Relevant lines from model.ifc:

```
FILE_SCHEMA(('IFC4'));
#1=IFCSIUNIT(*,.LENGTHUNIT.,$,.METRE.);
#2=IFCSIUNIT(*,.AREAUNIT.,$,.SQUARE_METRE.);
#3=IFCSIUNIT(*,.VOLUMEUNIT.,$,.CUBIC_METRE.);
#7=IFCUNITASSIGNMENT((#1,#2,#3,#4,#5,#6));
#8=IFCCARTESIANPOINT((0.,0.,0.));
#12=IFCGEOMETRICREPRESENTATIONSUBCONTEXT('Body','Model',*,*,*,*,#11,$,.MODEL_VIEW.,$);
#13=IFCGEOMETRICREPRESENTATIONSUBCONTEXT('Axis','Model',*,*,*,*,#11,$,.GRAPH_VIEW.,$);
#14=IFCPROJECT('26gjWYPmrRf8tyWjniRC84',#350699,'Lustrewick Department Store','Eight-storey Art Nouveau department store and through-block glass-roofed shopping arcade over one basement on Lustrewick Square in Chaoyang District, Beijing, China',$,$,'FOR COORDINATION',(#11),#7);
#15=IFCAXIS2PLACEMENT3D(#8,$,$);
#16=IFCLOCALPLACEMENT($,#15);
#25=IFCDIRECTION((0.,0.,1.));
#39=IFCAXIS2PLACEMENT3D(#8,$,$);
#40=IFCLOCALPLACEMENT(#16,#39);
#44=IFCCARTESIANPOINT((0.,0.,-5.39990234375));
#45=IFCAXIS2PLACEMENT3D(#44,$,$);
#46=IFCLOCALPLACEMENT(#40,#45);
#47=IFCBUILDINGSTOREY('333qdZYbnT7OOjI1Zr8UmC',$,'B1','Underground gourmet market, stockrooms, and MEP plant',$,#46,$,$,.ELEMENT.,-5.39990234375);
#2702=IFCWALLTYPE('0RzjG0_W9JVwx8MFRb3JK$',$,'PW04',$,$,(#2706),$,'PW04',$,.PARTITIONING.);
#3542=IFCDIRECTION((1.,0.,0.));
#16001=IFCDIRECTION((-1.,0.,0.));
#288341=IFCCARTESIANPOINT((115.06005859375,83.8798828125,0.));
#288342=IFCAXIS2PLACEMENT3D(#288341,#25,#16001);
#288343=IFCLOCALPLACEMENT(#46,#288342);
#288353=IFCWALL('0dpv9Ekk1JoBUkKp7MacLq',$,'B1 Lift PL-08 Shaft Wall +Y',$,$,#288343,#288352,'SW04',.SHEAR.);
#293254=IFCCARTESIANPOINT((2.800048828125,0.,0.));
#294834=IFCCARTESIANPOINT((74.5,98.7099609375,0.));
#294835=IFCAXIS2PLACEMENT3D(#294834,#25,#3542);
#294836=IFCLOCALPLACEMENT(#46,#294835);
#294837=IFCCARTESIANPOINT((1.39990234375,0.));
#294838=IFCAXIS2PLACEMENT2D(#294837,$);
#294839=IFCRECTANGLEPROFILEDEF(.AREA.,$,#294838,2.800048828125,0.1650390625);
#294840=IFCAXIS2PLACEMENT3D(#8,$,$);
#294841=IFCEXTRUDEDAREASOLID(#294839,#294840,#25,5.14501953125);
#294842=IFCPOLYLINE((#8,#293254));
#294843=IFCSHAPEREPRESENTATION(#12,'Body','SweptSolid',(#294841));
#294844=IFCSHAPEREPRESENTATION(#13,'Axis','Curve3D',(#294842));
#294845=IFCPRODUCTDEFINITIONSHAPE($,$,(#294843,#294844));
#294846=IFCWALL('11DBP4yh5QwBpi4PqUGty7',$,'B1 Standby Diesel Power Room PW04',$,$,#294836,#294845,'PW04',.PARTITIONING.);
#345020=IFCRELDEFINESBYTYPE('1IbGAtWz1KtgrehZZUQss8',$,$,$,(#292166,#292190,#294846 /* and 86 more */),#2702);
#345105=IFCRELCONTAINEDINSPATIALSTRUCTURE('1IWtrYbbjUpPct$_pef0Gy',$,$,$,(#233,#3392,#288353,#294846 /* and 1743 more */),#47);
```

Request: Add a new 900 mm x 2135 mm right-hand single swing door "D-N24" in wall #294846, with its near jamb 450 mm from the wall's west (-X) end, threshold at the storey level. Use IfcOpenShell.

```python
import numpy as np
import ifcopenshell
import ifcopenshell.api.feature
import ifcopenshell.api.geometry
import ifcopenshell.api.root
import ifcopenshell.api.spatial
import ifcopenshell.geom
import ifcopenshell.util.element
import ifcopenshell.util.placement
import ifcopenshell.util.representation
import ifcopenshell.util.shape
import ifcopenshell.util.unit

model = ifcopenshell.open("model.ifc")
unit_scale = ifcopenshell.util.unit.calculate_unit_scale(model)
settings = ifcopenshell.geom.settings()


def volume(element):
    """Net volume in cubic metres, openings subtracted."""
    shape = ifcopenshell.geom.create_shape(settings, element)
    return ifcopenshell.util.shape.get_volume(shape.geometry)


wall = model.by_guid("11DBP4yh5QwBpi4PqUGty7")
storey = ifcopenshell.util.element.get_container(wall, ifc_class="IfcBuildingStorey")
context = ifcopenshell.util.representation.get_context(model, "Model", "Body", "MODEL_VIEW")
before = volume(wall)

width, height, from_end, sill = 0.9, 2.135, 0.45, 0.0  # metres

# The wall runs along its own X axis, and the end named is its -X end.
wall_shape = ifcopenshell.geom.create_shape(settings, wall)
x, y, z = ifcopenshell.util.shape.get_vertices(wall_shape.geometry).T
start = x.min() + from_end
face, thickness = float(y.min()), float(y.max() - y.min())
wall_matrix = ifcopenshell.util.placement.get_local_placement(wall.ObjectPlacement)
level = ifcopenshell.util.placement.get_local_placement(storey.ObjectPlacement)[2, 3]


def in_wall(x, y):
    """Placement at x, y metres in the wall's axes, at sill height."""
    matrix = wall_matrix.copy()
    matrix[:, 3] = wall_matrix @ np.array([x / unit_scale, y / unit_scale, 0.0, 1.0])
    matrix[2, 3] = level + sill / unit_scale
    return matrix


# Opening: a box that overshoots both wall faces by 50 mm.
opening = ifcopenshell.api.root.create_entity(model, ifc_class="IfcOpeningElement", predefined_type="OPENING")
box = ifcopenshell.api.geometry.add_wall_representation(
    model, context=context, length=width, height=height, thickness=thickness + 0.1
)
ifcopenshell.api.geometry.assign_representation(model, product=opening, representation=box)
ifcopenshell.api.geometry.edit_object_placement(model, product=opening, matrix=in_wall(start, face - 0.05), is_si=False)
ifcopenshell.api.feature.add_feature(model, feature=opening, element=wall)

door = ifcopenshell.api.root.create_entity(model, ifc_class="IfcDoor", name="D-N24", predefined_type="DOOR")
door.OverallWidth, door.OverallHeight = width / unit_scale, height / unit_scale
door.OperationType = "SINGLE_SWING_RIGHT"
body = ifcopenshell.api.geometry.add_door_representation(
    model,
    context=context,
    overall_width=door.OverallWidth,
    overall_height=door.OverallHeight,
    operation_type="SINGLE_SWING_RIGHT",
    lining_properties={"LiningDepth": thickness / unit_scale, "ThresholdDepth": thickness / unit_scale},
)
ifcopenshell.api.geometry.assign_representation(model, product=door, representation=body)
ifcopenshell.api.spatial.assign_container(model, products=[door], relating_structure=storey)
ifcopenshell.api.feature.add_filling(model, opening=opening, element=door)

# The lining spans the wall, so the door starts at the wall face.
ifcopenshell.api.geometry.edit_object_placement(model, product=door, matrix=in_wall(start, face), is_si=False)

after = volume(wall)

print(f"wall volume {before:.3f} -> {after:.3f} m3")

model.write("model_edited.ifc")
```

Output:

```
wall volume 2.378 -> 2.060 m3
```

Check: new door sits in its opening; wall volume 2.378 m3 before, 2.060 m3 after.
